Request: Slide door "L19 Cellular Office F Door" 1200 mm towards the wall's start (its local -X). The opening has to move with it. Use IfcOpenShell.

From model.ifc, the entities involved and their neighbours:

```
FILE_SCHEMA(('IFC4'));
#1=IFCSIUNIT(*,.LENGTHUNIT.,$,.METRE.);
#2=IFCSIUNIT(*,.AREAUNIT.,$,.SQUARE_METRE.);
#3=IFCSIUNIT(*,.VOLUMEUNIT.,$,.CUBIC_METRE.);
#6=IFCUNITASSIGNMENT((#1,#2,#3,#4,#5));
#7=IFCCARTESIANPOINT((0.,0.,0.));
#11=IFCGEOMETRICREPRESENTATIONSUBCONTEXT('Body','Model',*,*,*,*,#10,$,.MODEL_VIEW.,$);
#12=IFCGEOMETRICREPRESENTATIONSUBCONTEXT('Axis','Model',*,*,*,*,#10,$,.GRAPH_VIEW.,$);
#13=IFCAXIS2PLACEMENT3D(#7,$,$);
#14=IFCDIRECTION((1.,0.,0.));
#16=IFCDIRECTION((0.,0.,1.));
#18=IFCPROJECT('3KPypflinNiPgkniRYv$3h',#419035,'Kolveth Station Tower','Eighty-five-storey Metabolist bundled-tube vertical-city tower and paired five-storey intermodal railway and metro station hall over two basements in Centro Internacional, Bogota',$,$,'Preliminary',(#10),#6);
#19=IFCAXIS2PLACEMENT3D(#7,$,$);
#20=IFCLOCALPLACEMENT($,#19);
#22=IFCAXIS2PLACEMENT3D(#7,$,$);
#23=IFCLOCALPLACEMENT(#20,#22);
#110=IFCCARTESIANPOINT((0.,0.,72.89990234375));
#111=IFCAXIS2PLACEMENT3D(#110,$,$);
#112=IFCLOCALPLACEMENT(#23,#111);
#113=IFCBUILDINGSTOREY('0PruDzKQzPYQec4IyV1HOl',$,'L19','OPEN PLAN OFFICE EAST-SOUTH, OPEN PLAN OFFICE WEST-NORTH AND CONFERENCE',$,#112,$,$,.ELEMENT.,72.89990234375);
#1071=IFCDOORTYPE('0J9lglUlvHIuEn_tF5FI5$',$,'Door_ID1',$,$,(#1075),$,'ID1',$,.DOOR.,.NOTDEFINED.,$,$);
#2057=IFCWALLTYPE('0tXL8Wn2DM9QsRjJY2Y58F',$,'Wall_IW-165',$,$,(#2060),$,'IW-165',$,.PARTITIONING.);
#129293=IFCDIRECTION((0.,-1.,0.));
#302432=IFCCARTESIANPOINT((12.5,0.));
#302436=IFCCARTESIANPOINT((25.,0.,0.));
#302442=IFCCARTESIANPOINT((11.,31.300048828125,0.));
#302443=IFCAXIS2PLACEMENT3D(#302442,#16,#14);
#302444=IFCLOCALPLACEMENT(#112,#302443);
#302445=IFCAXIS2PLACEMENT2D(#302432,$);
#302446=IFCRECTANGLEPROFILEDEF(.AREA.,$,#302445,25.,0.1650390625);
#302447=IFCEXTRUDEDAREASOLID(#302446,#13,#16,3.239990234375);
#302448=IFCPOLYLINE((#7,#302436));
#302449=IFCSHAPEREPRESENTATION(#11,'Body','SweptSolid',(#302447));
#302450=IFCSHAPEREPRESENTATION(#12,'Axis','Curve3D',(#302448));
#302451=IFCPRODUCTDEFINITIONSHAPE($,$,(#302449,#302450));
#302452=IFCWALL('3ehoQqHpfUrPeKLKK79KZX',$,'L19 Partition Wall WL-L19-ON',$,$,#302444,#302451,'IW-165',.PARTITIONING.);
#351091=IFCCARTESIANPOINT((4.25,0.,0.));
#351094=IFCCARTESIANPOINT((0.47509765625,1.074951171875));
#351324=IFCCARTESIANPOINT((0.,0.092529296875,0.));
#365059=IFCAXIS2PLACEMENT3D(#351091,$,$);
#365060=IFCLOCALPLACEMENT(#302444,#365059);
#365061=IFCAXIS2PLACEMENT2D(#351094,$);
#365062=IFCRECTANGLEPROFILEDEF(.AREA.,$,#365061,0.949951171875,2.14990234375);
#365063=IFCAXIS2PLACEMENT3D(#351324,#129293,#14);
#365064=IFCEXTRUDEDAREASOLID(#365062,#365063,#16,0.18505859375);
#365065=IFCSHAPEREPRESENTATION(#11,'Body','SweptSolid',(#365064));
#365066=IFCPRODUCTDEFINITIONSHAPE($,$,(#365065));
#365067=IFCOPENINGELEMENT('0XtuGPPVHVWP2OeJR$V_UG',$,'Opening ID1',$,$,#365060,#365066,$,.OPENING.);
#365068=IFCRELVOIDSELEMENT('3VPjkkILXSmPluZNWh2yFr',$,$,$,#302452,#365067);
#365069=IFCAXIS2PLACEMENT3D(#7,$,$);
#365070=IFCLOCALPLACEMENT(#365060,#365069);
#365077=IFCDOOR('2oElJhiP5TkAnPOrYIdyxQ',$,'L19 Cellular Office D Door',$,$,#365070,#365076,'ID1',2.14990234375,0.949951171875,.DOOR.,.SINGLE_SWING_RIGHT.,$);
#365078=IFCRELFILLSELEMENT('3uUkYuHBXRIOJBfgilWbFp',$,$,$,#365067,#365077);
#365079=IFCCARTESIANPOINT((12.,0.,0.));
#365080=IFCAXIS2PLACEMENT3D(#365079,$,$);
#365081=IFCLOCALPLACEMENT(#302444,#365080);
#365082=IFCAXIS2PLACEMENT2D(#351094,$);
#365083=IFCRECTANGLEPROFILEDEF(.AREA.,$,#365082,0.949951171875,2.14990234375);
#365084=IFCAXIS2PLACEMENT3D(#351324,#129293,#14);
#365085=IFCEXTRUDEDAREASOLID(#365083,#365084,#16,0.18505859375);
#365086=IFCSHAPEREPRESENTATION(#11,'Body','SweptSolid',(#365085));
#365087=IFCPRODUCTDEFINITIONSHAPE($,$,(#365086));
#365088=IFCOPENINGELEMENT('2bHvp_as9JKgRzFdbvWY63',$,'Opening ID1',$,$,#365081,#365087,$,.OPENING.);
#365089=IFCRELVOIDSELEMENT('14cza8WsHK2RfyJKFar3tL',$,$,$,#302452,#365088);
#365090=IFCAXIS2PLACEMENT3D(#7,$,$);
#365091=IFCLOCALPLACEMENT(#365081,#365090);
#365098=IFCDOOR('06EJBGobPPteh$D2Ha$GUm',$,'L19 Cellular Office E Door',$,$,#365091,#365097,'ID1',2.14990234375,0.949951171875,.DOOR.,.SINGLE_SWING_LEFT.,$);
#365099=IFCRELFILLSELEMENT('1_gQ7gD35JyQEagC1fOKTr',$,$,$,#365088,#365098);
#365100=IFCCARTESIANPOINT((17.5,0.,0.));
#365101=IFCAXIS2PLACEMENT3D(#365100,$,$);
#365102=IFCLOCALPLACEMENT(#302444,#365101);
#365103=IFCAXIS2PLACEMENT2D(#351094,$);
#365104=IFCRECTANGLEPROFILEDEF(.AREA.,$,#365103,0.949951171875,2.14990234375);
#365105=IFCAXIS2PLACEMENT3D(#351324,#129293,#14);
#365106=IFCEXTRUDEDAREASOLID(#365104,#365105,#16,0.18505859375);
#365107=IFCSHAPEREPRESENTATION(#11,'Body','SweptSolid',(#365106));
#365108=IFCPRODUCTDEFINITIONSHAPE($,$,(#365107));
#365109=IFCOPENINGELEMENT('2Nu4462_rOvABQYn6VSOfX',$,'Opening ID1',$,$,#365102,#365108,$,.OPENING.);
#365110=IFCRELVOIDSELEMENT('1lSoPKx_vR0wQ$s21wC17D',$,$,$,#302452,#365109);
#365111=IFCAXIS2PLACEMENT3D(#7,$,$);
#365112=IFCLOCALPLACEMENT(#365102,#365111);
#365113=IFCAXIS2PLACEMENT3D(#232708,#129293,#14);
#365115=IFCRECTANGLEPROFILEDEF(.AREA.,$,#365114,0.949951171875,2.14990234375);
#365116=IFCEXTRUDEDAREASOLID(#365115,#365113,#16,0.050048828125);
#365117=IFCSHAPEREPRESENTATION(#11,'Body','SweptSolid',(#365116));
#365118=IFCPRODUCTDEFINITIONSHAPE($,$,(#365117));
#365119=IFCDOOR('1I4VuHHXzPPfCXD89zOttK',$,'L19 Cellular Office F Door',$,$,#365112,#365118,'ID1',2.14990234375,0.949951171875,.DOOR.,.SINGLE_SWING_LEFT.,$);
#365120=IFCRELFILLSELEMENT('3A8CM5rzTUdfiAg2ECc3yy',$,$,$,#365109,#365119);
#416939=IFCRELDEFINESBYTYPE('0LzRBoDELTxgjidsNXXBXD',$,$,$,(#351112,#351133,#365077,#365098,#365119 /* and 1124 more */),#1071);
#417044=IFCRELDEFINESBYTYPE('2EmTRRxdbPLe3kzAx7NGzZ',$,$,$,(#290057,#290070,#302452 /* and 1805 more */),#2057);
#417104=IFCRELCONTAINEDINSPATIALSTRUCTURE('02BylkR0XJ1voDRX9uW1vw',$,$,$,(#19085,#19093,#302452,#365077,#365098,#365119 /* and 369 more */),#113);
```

```python
import ifcopenshell
import ifcopenshell.api.geometry
import ifcopenshell.util.placement
import ifcopenshell.util.unit

model = ifcopenshell.open("model.ifc")
unit_scale = ifcopenshell.util.unit.calculate_unit_scale(model)

door = model.by_guid("1I4VuHHXzPPfCXD89zOttK")
opening = door.FillsVoids[0].RelatingOpeningElement
wall = opening.VoidsElements[0].RelatingBuildingElement

wall_matrix = ifcopenshell.util.placement.get_local_placement(wall.ObjectPlacement)
shift = wall_matrix[:3, 0] * -1.2 / unit_scale
before = ifcopenshell.util.placement.get_local_placement(door.ObjectPlacement)[:3, 3].copy()

# The door is placed relative to its opening, so it follows when the opening moves.
matrix = ifcopenshell.util.placement.get_local_placement(opening.ObjectPlacement)
matrix[:3, 3] += shift
ifcopenshell.api.geometry.edit_object_placement(
    model, product=opening, matrix=matrix, is_si=False, should_transform_children=True
)

after = ifcopenshell.util.placement.get_local_placement(door.ObjectPlacement)[:3, 3]
print("door moved by", (after - before).round(3) + 0.0)

model.write("model_v2.ifc")
```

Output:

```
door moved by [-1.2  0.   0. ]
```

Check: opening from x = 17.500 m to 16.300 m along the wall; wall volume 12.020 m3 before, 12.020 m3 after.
